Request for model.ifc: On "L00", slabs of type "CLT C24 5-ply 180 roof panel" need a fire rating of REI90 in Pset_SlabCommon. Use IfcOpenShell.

First a look at what the model holds.

```python
import ifcopenshell
import ifcopenshell.util.element

model = ifcopenshell.open("model.ifc")
print(model.schema)
storey = next(s for s in model.by_type("IfcBuildingStorey") if s.Name == "L00")
slabs = [e for e in ifcopenshell.util.element.get_decomposition(storey) if e.is_a("IfcSlab")]
seen = {}
for e in slabs:
    element_type = ifcopenshell.util.element.get_type(e)
    key = (element_type.Name if element_type != e and element_type else None, ifcopenshell.util.element.get_pset(e, "Pset_SlabCommon", "FireRating"))
    seen[key] = seen.get(key, 0) + 1
for (name, value), count in sorted(seen.items(), key=str):
    print(count, "x", name, "|", value)
```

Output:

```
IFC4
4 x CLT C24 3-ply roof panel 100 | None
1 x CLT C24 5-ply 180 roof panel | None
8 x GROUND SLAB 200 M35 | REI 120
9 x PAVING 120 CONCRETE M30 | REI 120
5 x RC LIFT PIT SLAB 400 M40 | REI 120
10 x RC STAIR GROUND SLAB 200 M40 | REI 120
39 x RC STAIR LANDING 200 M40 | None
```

```python
import ifcopenshell
import ifcopenshell.api.pset
import ifcopenshell.util.element

model = ifcopenshell.open("model.ifc")

storey = next(s for s in model.by_type("IfcBuildingStorey") if s.Name == "L00")
slabs = [e for e in ifcopenshell.util.element.get_decomposition(storey) if e.is_a("IfcSlab")]

count = 0
for e in slabs:
    element_type = ifcopenshell.util.element.get_type(e)
    if element_type in (None, e) or element_type.Name != "CLT C24 5-ply 180 roof panel":
        continue
    # add_pset returns the element's existing set when there is one.
    pset = ifcopenshell.api.pset.add_pset(model, product=e, name="Pset_SlabCommon")
    ifcopenshell.api.pset.edit_pset(model, pset=pset, properties={"FireRating": "REI90"})
    count += 1

print(count, "slabs updated")

model.write("model_rev.ifc")
```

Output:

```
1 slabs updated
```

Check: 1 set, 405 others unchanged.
